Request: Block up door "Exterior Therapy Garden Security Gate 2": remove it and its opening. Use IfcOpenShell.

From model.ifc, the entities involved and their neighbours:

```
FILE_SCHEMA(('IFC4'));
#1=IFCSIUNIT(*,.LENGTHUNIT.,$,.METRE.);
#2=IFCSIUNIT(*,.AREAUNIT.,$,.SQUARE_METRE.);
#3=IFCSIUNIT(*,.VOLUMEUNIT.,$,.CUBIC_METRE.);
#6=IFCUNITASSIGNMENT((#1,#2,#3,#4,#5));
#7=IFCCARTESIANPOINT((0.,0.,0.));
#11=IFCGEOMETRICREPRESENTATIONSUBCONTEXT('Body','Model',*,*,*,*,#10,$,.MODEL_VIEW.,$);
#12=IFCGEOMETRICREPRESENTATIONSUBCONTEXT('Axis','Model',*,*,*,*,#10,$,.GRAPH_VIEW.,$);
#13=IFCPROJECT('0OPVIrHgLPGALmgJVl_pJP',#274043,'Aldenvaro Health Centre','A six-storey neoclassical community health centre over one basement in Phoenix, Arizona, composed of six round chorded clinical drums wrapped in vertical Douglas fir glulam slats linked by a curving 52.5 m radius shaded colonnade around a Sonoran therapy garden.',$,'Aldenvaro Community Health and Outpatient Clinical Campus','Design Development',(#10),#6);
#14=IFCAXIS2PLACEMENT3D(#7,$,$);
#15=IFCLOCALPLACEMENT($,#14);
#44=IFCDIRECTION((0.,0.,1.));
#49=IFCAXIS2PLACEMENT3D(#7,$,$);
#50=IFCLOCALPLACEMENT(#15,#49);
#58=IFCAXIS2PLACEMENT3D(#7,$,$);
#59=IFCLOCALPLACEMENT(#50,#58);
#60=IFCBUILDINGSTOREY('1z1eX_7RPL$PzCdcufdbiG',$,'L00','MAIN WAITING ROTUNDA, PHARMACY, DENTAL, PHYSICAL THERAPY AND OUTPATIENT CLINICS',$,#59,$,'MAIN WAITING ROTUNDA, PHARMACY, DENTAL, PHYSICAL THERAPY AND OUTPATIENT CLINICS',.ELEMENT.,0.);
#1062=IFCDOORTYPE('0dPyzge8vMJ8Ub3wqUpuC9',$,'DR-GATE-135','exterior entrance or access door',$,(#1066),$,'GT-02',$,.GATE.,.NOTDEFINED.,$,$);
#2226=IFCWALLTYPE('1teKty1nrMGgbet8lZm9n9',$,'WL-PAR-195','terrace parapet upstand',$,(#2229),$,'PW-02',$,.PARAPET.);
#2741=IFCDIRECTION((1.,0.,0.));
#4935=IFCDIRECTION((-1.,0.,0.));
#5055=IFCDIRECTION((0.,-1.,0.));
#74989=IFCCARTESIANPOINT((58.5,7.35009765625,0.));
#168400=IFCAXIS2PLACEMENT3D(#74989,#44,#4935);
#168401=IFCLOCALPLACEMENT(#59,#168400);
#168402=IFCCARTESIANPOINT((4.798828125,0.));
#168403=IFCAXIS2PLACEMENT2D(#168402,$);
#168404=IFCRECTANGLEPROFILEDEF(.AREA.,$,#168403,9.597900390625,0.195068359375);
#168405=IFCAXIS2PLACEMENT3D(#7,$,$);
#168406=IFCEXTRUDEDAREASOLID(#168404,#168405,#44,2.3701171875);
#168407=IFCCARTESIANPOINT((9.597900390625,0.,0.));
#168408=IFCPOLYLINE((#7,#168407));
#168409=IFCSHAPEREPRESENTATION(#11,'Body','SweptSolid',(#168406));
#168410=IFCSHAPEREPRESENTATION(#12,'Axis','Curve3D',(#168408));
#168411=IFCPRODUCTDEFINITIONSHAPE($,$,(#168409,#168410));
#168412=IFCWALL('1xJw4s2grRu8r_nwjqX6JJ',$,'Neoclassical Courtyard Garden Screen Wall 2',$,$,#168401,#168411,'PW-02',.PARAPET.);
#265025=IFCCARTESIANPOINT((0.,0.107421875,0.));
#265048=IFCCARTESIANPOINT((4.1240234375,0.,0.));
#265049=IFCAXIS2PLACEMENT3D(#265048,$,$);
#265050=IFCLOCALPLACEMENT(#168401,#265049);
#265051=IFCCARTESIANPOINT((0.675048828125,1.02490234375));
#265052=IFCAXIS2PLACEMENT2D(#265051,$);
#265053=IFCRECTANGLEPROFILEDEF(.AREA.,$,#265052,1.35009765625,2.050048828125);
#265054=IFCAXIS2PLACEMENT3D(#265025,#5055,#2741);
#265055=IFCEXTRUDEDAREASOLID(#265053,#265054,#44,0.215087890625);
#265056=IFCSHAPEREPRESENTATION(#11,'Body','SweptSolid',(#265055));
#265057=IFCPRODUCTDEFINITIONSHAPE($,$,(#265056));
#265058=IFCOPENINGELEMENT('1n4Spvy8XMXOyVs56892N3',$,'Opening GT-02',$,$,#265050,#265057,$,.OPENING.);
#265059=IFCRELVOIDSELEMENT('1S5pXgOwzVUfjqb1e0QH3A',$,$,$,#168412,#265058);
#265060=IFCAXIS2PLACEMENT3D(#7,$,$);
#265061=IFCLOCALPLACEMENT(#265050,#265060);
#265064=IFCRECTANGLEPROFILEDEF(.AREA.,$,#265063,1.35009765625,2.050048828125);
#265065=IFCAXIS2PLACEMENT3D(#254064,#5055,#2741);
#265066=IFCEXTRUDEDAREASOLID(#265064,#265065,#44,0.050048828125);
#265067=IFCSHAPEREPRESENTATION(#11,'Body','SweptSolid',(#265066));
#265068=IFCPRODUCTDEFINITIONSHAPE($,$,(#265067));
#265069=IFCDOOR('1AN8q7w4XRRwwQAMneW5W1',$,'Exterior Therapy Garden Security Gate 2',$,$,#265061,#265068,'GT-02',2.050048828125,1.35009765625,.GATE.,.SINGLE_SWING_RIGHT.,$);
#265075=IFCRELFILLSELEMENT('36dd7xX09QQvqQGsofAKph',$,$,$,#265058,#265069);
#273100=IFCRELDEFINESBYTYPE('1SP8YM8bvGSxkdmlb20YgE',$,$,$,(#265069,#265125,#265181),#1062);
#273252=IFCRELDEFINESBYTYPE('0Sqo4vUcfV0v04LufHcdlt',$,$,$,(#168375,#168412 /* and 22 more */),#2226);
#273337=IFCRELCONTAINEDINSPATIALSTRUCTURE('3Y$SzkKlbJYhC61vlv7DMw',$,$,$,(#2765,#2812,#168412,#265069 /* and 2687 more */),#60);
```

```python
import ifcopenshell
import ifcopenshell.api.feature
import ifcopenshell.api.root
import ifcopenshell.geom
import ifcopenshell.util.shape

model = ifcopenshell.open("model.ifc")
settings = ifcopenshell.geom.settings()


def volume(element):
    """Net volume in cubic metres, openings subtracted."""
    shape = ifcopenshell.geom.create_shape(settings, element)
    return ifcopenshell.util.shape.get_volume(shape.geometry)


door = model.by_guid("1AN8q7w4XRRwwQAMneW5W1")
opening = door.FillsVoids[0].RelatingOpeningElement
wall = opening.VoidsElements[0].RelatingBuildingElement
before = volume(wall)

ifcopenshell.api.root.remove_product(model, product=door)
ifcopenshell.api.feature.remove_feature(model, feature=opening)

after = volume(wall)

print(f"wall volume {before:.3f} -> {after:.3f} m3")

model.write("model_v2.ifc")
```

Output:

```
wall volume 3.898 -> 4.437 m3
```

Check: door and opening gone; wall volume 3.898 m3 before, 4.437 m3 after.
